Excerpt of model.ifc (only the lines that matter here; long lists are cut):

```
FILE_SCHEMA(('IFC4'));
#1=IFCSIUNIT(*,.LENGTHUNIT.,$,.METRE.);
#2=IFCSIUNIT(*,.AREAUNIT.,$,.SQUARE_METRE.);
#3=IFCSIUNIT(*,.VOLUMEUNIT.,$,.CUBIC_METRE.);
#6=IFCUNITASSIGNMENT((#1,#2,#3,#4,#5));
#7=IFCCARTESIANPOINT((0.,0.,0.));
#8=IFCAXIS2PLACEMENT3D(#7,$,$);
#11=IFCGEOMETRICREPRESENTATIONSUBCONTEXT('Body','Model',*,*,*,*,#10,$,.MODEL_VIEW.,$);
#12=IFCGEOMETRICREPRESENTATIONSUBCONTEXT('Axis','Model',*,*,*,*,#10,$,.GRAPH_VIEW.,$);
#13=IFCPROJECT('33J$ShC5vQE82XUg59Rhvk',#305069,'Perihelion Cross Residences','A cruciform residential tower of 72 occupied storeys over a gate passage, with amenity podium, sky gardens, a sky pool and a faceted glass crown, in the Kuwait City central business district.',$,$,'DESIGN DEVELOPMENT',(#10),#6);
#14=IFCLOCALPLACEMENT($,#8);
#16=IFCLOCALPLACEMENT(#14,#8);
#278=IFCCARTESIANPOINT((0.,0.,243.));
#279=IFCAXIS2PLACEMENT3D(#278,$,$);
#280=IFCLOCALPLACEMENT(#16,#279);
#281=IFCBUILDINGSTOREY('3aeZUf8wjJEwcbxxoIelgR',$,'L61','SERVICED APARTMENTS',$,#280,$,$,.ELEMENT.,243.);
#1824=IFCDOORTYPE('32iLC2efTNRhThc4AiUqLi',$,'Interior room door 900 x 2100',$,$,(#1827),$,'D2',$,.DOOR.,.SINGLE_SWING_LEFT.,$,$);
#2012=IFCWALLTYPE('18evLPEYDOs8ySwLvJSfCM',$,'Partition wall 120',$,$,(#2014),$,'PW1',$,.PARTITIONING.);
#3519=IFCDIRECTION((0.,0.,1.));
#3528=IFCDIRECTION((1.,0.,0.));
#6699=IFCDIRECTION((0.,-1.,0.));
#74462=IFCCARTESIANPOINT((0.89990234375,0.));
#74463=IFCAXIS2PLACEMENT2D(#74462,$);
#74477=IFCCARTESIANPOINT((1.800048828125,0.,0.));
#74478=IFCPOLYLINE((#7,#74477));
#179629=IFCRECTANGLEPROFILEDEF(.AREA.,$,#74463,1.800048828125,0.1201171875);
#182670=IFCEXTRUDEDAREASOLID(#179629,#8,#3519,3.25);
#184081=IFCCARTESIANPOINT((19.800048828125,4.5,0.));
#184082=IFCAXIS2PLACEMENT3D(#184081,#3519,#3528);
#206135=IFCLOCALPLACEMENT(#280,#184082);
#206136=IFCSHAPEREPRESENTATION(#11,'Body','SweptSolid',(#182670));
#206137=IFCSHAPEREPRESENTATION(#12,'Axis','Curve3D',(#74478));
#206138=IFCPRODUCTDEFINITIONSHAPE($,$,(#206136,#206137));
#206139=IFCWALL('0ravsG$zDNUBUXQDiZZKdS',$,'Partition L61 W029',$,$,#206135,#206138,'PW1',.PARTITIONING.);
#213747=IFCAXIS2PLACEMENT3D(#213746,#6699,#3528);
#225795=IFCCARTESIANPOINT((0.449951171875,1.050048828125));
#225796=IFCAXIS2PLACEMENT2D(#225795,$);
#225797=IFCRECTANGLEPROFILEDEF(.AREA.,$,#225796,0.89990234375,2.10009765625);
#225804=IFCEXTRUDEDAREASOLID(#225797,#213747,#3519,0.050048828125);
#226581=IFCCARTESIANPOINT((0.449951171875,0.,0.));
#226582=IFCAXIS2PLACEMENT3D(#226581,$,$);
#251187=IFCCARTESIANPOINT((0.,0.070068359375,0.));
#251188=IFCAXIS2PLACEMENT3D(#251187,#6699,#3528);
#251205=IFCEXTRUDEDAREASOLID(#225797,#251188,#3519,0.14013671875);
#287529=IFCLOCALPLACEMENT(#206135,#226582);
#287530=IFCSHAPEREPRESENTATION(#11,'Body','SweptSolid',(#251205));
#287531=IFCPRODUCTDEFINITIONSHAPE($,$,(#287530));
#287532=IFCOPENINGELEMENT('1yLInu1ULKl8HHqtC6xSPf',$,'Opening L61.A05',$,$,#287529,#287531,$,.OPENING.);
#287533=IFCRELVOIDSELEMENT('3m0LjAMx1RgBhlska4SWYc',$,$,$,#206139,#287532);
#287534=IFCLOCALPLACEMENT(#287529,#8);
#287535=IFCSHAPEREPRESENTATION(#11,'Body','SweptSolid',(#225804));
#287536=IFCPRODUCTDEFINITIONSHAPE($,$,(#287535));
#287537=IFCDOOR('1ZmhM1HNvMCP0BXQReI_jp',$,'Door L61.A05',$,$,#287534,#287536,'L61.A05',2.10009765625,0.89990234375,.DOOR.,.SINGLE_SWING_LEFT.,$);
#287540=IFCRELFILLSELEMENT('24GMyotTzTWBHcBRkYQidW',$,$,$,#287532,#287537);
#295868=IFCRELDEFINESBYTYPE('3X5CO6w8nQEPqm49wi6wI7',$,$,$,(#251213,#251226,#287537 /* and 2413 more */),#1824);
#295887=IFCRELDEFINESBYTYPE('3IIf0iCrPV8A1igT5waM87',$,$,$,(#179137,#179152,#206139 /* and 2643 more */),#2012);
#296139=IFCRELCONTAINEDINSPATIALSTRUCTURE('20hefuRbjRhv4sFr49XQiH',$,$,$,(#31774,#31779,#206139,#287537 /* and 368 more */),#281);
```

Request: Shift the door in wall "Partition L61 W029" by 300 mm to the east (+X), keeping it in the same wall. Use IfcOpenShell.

```python
import ifcopenshell
import ifcopenshell.api.geometry
import ifcopenshell.util.placement

model = ifcopenshell.open("model.ifc")

door = model.by_guid("1ZmhM1HNvMCP0BXQReI_jp")
opening = door.FillsVoids[0].RelatingOpeningElement
wall = opening.VoidsElements[0].RelatingBuildingElement

wall_matrix = ifcopenshell.util.placement.get_local_placement(wall.ObjectPlacement)
shift = wall_matrix[:3, 0] * 0.3
before = ifcopenshell.util.placement.get_local_placement(door.ObjectPlacement)[:3, 3].copy()

# The door is placed relative to its opening, so it follows when the opening moves.
matrix = ifcopenshell.util.placement.get_local_placement(opening.ObjectPlacement)
matrix[:3, 3] += shift
ifcopenshell.api.geometry.edit_object_placement(
    model, product=opening, matrix=matrix, is_si=False, should_transform_children=True
)

after = ifcopenshell.util.placement.get_local_placement(door.ObjectPlacement)[:3, 3]
print("door moved by", (after - before).round(3) + 0.0)

model.write("model_v2.ifc")
```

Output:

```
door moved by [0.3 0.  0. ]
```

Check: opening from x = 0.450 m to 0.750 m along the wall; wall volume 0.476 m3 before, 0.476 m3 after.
